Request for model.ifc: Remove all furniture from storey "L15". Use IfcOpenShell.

First a look at what the model holds.

```python
import ifcopenshell
import ifcopenshell.util.element

model = ifcopenshell.open("model.ifc")
print(model.schema)
storey = next(s for s in model.by_type("IfcBuildingStorey") if s.Name == "L15")
furniture = [e for e in ifcopenshell.util.element.get_decomposition(storey) if e.is_a("IfcFurnishingElement")]
seen = {}
for e in furniture:
    element_type = ifcopenshell.util.element.get_type(e)
    name = element_type.Name if element_type not in (None, e) else None
    seen[name] = seen.get(name, 0) + 1
for name, count in sorted(seen.items(), key=str):
    print(count, "x", name)
```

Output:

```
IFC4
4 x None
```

```python
import ifcopenshell
import ifcopenshell.api.root
import ifcopenshell.util.element

model = ifcopenshell.open("model.ifc")

storey = next(s for s in model.by_type("IfcBuildingStorey") if s.Name == "L15")
furniture = [e for e in ifcopenshell.util.element.get_decomposition(storey) if e.is_a("IfcFurnishingElement")]

for e in furniture:
    ifcopenshell.api.root.remove_product(model, product=e)
print(len(furniture), "removed")

model.write("model_rev.ifc")
```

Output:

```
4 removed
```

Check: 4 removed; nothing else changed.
